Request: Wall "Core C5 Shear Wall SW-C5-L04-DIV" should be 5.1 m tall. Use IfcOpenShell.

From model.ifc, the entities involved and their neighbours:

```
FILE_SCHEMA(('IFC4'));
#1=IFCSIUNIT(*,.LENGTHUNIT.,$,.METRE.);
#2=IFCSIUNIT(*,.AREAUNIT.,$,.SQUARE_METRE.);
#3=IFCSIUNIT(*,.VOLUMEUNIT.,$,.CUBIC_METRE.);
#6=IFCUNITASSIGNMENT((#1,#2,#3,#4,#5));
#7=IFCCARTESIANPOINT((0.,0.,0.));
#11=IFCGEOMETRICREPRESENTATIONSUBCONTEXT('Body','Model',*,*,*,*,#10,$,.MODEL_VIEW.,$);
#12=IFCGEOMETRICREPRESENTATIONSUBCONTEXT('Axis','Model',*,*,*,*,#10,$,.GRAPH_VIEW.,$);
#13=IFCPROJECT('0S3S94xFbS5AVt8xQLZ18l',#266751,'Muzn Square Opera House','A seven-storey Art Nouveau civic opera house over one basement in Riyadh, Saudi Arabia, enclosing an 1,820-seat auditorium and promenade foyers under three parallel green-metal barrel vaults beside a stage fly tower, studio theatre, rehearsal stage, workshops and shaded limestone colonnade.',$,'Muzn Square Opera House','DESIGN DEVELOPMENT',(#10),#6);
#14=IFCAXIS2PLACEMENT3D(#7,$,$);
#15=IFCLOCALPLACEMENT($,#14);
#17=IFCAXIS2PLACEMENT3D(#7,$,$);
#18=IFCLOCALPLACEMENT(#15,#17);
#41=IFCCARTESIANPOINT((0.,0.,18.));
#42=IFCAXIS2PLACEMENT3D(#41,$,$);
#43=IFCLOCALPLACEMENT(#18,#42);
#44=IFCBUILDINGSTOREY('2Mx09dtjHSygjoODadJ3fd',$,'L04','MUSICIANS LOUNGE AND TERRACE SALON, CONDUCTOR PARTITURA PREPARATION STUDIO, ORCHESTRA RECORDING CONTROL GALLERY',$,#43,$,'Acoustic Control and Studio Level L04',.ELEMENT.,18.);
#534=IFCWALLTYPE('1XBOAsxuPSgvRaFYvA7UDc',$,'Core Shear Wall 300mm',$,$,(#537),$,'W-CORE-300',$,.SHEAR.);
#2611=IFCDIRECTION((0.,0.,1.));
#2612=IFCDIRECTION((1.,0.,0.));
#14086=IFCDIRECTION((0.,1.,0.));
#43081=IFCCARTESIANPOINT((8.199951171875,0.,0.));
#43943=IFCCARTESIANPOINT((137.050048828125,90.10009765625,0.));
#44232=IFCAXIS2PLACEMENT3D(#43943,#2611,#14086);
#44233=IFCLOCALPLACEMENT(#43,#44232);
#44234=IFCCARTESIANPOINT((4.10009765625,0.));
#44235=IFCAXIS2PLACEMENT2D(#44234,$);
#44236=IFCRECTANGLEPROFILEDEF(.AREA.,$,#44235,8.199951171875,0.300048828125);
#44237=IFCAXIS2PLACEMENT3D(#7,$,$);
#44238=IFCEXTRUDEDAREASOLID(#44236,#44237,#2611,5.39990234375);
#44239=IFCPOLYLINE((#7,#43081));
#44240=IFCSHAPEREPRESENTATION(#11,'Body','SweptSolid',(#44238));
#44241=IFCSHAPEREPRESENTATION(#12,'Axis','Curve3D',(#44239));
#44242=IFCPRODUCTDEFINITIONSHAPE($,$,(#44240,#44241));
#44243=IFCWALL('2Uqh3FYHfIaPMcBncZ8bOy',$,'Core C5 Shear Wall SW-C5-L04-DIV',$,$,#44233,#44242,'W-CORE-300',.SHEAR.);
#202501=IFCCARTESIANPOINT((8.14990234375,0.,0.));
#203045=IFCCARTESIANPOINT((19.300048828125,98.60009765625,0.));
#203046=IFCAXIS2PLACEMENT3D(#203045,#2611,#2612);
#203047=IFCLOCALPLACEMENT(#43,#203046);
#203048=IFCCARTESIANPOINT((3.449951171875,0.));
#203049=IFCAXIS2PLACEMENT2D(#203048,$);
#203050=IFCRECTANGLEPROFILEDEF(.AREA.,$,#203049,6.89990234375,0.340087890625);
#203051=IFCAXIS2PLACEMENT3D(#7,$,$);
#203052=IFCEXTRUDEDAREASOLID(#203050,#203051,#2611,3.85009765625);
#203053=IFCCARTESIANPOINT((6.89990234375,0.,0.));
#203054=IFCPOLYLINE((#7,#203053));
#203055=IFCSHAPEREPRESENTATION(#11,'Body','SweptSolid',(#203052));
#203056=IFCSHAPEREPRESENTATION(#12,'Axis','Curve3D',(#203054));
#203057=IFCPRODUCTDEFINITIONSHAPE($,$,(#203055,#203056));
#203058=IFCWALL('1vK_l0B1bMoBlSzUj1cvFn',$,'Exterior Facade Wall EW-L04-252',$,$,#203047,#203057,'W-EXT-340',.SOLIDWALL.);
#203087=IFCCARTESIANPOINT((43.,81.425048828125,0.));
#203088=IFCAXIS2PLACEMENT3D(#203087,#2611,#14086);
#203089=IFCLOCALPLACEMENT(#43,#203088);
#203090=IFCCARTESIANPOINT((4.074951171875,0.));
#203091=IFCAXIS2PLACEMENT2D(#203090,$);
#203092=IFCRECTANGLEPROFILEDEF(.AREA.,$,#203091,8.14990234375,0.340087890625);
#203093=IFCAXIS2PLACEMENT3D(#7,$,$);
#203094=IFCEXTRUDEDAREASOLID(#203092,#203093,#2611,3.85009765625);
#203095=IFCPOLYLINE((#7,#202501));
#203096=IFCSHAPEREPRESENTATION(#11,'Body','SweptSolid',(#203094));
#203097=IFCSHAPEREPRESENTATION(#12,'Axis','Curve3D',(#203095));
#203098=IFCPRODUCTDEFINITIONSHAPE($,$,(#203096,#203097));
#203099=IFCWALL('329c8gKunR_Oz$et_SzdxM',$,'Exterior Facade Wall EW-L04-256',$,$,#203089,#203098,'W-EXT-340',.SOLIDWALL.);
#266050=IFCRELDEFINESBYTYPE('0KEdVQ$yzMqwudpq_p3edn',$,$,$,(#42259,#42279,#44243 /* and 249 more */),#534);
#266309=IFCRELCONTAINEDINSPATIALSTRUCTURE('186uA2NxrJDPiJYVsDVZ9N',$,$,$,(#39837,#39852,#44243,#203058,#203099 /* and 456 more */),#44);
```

```python
import ifcopenshell
import ifcopenshell.geom
import ifcopenshell.util.representation
import ifcopenshell.util.shape

model = ifcopenshell.open("model.ifc")
settings = ifcopenshell.geom.settings()


def volume(element):
    """Net volume in cubic metres, openings subtracted."""
    shape = ifcopenshell.geom.create_shape(settings, element)
    return ifcopenshell.util.shape.get_volume(shape.geometry)


wall = model.by_id(44243)
before = volume(wall)

body = ifcopenshell.util.representation.get_representation(wall, "Model", "Body")
solid = body.Items[0]
old_height = solid.Depth
solid.Depth = 5.1
after = volume(wall)

print(f"height {old_height:g} -> {solid.Depth:g}, volume {before:.3f} -> {after:.3f} m3")

model.write("model_edited.ifc")
```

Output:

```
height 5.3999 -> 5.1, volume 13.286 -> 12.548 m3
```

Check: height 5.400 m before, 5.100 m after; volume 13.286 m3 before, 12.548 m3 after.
